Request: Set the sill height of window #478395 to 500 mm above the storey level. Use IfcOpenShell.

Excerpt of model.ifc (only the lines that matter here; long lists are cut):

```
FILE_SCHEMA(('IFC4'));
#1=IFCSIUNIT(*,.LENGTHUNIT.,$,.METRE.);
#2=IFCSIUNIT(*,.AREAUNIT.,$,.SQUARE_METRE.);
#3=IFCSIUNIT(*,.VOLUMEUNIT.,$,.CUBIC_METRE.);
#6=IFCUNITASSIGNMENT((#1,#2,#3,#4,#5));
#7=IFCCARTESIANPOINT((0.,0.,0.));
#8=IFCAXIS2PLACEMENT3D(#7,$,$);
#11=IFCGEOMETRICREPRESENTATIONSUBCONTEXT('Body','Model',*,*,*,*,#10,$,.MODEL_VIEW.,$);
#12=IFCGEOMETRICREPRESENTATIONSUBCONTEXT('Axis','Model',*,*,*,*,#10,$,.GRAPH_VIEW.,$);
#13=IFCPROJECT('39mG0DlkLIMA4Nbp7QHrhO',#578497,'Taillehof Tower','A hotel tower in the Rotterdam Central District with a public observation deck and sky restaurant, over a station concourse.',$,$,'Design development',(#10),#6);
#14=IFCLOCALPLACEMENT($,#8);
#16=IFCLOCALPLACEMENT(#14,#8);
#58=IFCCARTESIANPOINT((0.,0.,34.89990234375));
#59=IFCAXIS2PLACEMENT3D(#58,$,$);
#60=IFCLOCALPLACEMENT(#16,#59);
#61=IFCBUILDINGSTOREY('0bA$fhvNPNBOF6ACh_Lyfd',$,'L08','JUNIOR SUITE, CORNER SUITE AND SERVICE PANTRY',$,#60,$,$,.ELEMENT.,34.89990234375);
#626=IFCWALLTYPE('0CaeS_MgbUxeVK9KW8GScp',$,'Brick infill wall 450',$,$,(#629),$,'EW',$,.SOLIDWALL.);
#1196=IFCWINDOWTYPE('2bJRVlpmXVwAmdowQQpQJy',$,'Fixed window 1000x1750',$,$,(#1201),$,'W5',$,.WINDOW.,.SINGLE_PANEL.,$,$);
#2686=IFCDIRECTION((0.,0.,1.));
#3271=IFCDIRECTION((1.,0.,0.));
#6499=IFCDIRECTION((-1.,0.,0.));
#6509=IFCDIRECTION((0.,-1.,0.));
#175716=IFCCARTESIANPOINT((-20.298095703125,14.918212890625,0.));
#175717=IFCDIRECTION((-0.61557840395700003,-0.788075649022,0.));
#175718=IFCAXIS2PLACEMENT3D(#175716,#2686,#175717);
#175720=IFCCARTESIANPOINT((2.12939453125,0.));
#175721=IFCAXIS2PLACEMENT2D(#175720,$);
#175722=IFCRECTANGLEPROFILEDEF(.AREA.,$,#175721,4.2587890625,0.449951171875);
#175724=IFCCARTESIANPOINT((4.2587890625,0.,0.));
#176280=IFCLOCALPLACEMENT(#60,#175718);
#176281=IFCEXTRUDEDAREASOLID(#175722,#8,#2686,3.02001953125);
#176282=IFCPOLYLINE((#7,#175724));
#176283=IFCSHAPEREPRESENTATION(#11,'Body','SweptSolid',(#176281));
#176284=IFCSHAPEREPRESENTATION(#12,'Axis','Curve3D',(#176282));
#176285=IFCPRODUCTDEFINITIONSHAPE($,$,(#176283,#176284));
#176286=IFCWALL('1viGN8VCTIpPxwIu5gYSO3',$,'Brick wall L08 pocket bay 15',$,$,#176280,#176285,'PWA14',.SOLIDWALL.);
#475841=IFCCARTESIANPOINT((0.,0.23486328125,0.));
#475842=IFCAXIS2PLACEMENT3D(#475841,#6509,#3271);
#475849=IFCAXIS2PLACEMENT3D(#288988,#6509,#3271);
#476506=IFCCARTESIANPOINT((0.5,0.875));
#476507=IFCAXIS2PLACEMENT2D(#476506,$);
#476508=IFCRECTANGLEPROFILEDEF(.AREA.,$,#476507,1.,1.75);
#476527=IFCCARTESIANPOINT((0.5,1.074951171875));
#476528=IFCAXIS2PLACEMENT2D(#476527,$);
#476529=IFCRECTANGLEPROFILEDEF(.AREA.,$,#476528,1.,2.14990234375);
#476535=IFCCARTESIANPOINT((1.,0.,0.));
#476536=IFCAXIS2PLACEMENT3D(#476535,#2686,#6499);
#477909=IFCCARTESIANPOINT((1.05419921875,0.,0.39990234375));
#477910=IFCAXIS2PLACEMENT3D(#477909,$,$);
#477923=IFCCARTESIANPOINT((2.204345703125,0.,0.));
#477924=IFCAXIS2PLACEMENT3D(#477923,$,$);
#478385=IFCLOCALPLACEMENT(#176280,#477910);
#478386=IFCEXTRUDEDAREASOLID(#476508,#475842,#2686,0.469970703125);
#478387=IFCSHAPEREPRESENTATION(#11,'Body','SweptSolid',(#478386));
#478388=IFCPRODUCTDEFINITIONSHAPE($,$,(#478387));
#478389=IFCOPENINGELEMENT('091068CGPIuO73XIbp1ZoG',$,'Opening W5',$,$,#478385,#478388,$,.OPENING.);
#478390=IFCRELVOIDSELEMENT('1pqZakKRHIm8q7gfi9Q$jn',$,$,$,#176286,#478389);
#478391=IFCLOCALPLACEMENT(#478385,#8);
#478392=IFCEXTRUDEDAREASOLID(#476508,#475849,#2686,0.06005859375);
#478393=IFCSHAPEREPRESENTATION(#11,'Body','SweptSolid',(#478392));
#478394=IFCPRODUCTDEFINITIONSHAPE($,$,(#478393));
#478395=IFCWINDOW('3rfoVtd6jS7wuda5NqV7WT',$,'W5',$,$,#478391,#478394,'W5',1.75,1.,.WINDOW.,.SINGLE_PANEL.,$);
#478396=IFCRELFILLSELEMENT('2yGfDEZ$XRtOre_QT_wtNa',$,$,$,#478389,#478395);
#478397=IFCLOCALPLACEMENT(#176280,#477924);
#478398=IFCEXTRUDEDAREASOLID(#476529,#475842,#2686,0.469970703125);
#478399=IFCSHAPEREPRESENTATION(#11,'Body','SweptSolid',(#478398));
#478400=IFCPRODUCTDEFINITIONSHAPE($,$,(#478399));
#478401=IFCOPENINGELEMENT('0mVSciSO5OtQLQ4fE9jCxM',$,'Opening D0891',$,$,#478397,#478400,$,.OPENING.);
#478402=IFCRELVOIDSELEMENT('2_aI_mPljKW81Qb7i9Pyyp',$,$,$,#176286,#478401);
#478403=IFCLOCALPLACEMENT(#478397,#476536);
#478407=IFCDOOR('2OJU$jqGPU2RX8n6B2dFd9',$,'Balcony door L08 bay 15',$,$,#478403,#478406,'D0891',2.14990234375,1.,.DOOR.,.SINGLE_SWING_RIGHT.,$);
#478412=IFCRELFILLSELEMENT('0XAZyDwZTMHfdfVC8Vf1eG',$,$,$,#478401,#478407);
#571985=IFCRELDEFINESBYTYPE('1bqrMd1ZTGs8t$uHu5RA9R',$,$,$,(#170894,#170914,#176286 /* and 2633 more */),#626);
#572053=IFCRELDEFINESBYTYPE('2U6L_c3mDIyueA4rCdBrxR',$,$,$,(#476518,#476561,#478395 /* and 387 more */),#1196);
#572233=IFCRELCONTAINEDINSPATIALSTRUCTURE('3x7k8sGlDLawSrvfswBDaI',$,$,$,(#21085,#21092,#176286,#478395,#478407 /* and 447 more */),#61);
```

```python
import numpy as np
import ifcopenshell
import ifcopenshell.api.geometry
import ifcopenshell.geom
import ifcopenshell.util.element
import ifcopenshell.util.placement
import ifcopenshell.util.shape
import ifcopenshell.util.unit

model = ifcopenshell.open("model.ifc")
unit_scale = ifcopenshell.util.unit.calculate_unit_scale(model)

window = model.by_guid("3rfoVtd6jS7wuda5NqV7WT")
opening = window.FillsVoids[0].RelatingOpeningElement
storey = ifcopenshell.util.element.get_container(window, ifc_class="IfcBuildingStorey")
level = ifcopenshell.util.placement.get_local_placement(storey.ObjectPlacement)[2, 3]

# The opening's origin need not be at the sill, so measure its lowest point.
shape = ifcopenshell.geom.create_shape(ifcopenshell.geom.settings(), opening)
bottom = ifcopenshell.util.shape.get_shape_bottom_elevation(shape, shape.geometry) / unit_scale
dz = level + 0.5 / unit_scale - bottom

shift = np.array([0.0, 0.0, dz])
# The window is placed relative to its opening, so it follows when the opening moves.
matrix = ifcopenshell.util.placement.get_local_placement(opening.ObjectPlacement)
matrix[:3, 3] += shift
ifcopenshell.api.geometry.edit_object_placement(
    model, product=opening, matrix=matrix, is_si=False, should_transform_children=True
)

print(f"moved by {dz * unit_scale:+.3f} m")

model.write("model_edited.ifc")
```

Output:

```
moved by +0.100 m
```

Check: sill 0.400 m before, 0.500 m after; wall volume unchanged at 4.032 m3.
